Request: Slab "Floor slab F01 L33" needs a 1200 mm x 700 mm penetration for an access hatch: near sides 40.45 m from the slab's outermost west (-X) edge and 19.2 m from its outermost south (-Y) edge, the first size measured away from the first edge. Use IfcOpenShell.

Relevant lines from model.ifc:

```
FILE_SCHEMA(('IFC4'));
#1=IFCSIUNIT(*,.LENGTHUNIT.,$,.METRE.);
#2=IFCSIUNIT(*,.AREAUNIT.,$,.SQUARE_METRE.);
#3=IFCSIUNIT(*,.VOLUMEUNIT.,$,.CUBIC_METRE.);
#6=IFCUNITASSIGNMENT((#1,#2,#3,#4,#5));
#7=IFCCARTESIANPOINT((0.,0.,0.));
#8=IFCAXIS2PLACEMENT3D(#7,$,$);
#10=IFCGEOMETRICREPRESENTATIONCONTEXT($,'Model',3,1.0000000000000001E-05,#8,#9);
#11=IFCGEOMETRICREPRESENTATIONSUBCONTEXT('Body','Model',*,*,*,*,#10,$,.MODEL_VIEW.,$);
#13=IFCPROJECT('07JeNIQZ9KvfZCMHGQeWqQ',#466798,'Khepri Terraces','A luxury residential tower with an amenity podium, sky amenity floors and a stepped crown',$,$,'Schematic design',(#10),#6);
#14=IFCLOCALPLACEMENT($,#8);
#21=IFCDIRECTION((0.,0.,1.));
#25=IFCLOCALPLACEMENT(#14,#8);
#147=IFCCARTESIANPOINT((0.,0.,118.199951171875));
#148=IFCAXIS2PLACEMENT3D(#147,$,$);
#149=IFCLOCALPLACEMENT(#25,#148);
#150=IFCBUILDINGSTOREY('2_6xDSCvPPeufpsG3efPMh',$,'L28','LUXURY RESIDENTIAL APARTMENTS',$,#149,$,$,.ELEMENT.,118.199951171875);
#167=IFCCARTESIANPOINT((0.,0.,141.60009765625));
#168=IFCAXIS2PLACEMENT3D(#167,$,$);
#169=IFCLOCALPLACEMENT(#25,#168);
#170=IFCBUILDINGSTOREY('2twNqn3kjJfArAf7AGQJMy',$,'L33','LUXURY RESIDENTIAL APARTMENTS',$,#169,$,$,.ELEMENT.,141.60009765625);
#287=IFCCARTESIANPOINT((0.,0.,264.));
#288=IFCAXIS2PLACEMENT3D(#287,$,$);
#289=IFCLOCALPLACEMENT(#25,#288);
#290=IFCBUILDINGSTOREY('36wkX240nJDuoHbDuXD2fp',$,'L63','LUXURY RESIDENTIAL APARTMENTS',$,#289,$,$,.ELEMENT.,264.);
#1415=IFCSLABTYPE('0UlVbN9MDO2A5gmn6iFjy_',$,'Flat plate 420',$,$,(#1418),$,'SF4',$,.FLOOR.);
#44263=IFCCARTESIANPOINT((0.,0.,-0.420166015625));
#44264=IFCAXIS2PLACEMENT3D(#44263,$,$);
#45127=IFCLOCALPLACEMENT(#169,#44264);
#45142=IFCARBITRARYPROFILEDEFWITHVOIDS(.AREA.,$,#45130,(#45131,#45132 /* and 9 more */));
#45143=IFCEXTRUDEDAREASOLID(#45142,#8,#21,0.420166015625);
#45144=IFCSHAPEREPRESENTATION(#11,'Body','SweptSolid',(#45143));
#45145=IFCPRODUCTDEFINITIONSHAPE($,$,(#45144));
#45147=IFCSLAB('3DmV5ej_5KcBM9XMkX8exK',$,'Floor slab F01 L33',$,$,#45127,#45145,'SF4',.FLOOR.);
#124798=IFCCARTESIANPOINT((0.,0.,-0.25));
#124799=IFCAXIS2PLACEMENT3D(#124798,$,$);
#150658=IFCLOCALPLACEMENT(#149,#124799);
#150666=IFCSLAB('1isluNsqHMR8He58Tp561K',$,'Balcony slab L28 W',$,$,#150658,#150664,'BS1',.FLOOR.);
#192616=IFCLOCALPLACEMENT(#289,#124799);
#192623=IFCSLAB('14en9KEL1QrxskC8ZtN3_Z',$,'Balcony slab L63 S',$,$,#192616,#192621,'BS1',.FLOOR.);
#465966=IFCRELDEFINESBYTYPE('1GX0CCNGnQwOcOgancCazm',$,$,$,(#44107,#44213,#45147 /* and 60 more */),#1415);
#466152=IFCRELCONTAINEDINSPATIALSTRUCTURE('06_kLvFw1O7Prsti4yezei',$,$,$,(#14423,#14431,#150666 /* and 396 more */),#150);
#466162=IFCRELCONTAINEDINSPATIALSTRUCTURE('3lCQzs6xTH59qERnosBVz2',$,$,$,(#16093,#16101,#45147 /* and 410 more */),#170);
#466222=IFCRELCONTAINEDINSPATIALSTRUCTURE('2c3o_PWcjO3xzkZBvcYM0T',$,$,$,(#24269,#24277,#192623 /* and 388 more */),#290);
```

```python
import numpy as np
import ifcopenshell
import ifcopenshell.api.feature
import ifcopenshell.api.geometry
import ifcopenshell.api.root
import ifcopenshell.geom
import ifcopenshell.util.placement
import ifcopenshell.util.representation
import ifcopenshell.util.shape
import ifcopenshell.util.unit

model = ifcopenshell.open("model.ifc")
unit_scale = ifcopenshell.util.unit.calculate_unit_scale(model)
settings = ifcopenshell.geom.settings()


def volume(element):
    """Net volume in cubic metres, openings subtracted."""
    shape = ifcopenshell.geom.create_shape(settings, element)
    return ifcopenshell.util.shape.get_volume(shape.geometry)


slab = model.by_id(45147)
before = volume(slab)

# Extent in the slab's own axes, in metres. The edges named are its -X and -Y sides.
slab_shape = ifcopenshell.geom.create_shape(settings, slab)
vertices = ifcopenshell.util.shape.get_vertices(slab_shape.geometry)
x_min, y_min, bottom = vertices.min(axis=0)
top = vertices[:, 2].max()

opening = ifcopenshell.api.root.create_entity(model, ifc_class="IfcOpeningElement", name="Access hatch opening", predefined_type="OPENING")
context = ifcopenshell.util.representation.get_context(model, "Model", "Body", "MODEL_VIEW")
width, depth = 1.2, 0.7
outline = [(0.0, 0.0), (width, 0.0), (width, depth), (0.0, depth), (0.0, 0.0)]
# Overshoot both faces by 50 mm so the cut is clean.
shape = ifcopenshell.api.geometry.add_slab_representation(
    model, context=context, depth=top - bottom + 0.1, polyline=outline
)
ifcopenshell.api.geometry.assign_representation(model, product=opening, representation=shape)

matrix = ifcopenshell.util.placement.get_local_placement(slab.ObjectPlacement)
matrix[:, 3] = matrix @ np.append(np.array([x_min + 40.45, y_min + 19.2, bottom - 0.05]) / unit_scale, 1.0)
ifcopenshell.api.geometry.edit_object_placement(model, product=opening, matrix=matrix, is_si=False)
ifcopenshell.api.feature.add_feature(model, feature=opening, element=slab)

after = volume(slab)

print(f"slab volume {before:.3f} -> {after:.3f} m3")

model.write("model_edited.ifc")
```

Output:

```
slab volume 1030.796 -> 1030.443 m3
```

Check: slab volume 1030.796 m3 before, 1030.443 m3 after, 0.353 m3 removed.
